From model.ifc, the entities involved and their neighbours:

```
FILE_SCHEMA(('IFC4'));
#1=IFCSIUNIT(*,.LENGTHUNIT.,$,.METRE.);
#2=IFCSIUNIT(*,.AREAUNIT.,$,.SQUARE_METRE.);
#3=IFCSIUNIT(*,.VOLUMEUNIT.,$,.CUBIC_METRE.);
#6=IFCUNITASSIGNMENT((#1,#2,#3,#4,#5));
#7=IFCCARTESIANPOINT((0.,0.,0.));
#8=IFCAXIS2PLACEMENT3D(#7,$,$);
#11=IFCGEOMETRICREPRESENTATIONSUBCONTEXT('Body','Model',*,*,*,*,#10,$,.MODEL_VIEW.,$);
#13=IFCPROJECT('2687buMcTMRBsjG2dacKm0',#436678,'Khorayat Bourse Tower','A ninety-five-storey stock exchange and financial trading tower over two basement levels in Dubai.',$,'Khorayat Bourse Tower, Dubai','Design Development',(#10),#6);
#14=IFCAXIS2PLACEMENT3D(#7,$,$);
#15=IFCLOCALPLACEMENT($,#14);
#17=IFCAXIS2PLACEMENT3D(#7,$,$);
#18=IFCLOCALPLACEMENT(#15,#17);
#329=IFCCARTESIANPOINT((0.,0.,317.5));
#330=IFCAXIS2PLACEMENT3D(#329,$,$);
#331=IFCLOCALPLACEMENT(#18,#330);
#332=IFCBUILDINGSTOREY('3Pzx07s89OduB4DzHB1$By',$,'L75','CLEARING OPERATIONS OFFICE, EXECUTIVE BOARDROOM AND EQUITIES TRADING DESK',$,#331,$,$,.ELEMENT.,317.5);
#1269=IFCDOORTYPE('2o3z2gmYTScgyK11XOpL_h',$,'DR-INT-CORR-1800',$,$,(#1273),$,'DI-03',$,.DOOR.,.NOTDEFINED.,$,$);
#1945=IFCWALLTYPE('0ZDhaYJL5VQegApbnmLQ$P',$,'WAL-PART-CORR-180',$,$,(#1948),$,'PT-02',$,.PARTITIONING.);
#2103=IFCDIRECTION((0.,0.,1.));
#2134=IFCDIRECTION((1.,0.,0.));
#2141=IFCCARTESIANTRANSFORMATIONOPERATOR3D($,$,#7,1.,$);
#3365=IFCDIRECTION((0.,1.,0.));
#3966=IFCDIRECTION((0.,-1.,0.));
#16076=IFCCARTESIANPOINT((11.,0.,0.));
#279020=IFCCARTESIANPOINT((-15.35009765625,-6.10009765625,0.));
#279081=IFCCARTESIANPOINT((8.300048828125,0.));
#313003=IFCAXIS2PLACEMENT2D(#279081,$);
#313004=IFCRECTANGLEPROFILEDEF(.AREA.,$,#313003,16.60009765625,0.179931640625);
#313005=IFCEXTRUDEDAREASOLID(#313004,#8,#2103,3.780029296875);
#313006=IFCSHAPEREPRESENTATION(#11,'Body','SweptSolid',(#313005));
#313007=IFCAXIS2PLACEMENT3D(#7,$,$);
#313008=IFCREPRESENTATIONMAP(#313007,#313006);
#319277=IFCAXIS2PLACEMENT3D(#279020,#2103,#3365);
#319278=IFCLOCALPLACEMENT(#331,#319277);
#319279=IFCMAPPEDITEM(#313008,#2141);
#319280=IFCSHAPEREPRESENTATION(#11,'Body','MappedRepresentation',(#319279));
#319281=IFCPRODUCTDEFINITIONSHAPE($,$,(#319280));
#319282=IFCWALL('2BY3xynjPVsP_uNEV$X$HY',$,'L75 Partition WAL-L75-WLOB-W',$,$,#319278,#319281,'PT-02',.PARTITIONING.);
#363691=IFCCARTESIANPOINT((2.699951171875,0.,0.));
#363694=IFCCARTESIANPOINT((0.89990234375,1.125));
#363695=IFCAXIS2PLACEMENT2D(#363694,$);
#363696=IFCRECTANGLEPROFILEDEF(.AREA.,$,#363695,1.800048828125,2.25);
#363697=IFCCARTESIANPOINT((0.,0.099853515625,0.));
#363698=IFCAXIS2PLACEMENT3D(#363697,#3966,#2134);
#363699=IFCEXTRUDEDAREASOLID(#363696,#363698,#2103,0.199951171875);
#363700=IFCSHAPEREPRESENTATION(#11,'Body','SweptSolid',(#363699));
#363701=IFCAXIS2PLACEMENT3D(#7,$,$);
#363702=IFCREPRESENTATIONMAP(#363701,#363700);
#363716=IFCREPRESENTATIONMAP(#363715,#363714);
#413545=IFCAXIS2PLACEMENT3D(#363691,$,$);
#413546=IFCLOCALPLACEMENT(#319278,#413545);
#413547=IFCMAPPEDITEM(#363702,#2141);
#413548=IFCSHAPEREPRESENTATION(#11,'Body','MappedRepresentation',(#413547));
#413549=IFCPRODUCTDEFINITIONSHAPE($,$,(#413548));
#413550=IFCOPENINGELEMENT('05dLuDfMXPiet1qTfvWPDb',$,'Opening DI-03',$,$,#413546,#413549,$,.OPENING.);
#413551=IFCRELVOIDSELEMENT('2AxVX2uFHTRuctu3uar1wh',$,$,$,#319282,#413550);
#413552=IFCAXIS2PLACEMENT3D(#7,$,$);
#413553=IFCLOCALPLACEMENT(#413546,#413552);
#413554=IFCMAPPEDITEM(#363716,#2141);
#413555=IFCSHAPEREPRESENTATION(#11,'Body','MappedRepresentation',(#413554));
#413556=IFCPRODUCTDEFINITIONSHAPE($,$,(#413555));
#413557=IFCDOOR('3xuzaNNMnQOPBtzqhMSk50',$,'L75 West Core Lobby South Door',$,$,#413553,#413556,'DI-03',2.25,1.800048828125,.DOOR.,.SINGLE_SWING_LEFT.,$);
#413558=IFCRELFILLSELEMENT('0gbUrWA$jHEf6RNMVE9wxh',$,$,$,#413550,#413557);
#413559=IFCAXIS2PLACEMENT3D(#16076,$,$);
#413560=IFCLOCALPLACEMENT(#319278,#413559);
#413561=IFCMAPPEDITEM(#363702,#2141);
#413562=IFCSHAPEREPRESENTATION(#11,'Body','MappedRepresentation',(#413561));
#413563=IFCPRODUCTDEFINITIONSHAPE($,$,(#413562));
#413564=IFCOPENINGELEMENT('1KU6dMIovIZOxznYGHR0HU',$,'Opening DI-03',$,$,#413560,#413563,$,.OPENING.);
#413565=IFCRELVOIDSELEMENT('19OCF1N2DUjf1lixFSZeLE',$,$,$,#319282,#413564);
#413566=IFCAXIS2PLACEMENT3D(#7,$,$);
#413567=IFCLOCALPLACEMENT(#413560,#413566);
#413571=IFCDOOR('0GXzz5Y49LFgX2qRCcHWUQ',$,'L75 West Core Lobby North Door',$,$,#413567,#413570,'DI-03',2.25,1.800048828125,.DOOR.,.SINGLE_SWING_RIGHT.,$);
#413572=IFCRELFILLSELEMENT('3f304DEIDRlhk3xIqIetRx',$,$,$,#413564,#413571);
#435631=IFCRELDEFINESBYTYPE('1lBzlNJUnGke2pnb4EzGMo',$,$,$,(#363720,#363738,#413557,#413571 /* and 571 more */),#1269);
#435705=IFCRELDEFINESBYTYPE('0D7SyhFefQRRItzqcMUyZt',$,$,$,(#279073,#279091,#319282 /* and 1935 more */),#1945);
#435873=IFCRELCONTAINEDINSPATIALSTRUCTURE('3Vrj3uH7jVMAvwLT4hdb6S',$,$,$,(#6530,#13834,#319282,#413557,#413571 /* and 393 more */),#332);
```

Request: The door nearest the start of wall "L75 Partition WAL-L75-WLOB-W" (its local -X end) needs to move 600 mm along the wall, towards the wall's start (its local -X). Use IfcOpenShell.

```python
import ifcopenshell
import ifcopenshell.api.geometry
import ifcopenshell.util.placement
import ifcopenshell.util.unit

model = ifcopenshell.open("model.ifc")
unit_scale = ifcopenshell.util.unit.calculate_unit_scale(model)

door = model.by_id(413557)
opening = door.FillsVoids[0].RelatingOpeningElement
wall = opening.VoidsElements[0].RelatingBuildingElement

wall_matrix = ifcopenshell.util.placement.get_local_placement(wall.ObjectPlacement)
shift = wall_matrix[:3, 0] * -0.6 / unit_scale
before = ifcopenshell.util.placement.get_local_placement(door.ObjectPlacement)[:3, 3].copy()

# The door is placed relative to its opening, so it follows when the opening moves.
matrix = ifcopenshell.util.placement.get_local_placement(opening.ObjectPlacement)
matrix[:3, 3] += shift
ifcopenshell.api.geometry.edit_object_placement(
    model, product=opening, matrix=matrix, is_si=False, should_transform_children=True
)

after = ifcopenshell.util.placement.get_local_placement(door.ObjectPlacement)[:3, 3]
print("door moved by", (after - before).round(3) + 0.0)

model.write("model_updated.ifc")
```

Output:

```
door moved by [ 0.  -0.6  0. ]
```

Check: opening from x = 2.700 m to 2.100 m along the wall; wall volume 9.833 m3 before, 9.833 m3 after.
